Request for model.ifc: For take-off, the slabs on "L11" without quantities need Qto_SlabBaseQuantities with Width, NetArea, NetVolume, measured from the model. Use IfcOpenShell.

First a look at what the model holds.

```python
import ifcopenshell
import ifcopenshell.util.element
import ifcopenshell.util.unit

model = ifcopenshell.open("model.ifc")
print(model.schema)
for unit_type in ("LENGTHUNIT", "AREAUNIT", "VOLUMEUNIT"):
    print(unit_type, ifcopenshell.util.unit.calculate_unit_scale(model, unit_type))
storey = next(s for s in model.by_type("IfcBuildingStorey") if s.Name == "L11")
slabs = [e for e in ifcopenshell.util.element.get_decomposition(storey) if e.is_a("IfcSlab")]
for e in sorted(slabs, key=lambda e: e.id()):
    print(e.id(), e.is_a(), e.Name, list(ifcopenshell.util.element.get_psets(e, qtos_only=True)), sep=" | ")
```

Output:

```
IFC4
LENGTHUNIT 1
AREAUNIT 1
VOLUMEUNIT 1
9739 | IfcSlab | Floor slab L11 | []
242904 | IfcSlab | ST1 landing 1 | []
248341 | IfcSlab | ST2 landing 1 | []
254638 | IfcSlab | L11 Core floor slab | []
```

```python
import ifcopenshell
import ifcopenshell.api.pset
import ifcopenshell.geom
import ifcopenshell.util.element
import ifcopenshell.util.shape
import ifcopenshell.util.unit

model = ifcopenshell.open("model.ifc")
unit_scale = ifcopenshell.util.unit.calculate_unit_scale(model)
area_scale = ifcopenshell.util.unit.calculate_unit_scale(model, "AREAUNIT")
volume_scale = ifcopenshell.util.unit.calculate_unit_scale(model, "VOLUMEUNIT")
settings = ifcopenshell.geom.settings()

storey = next(s for s in model.by_type("IfcBuildingStorey") if s.Name == "L11")
slabs = [e for e in ifcopenshell.util.element.get_decomposition(storey) if e.is_a("IfcSlab")]

for e in sorted(slabs, key=lambda e: e.id()):
    if ifcopenshell.util.element.get_psets(e, qtos_only=True, should_inherit=False):
        continue
    # Geometry comes back in metres, in the element's own axes.
    shape = ifcopenshell.geom.create_shape(settings, e)
    values = {
        "Width": ifcopenshell.util.shape.get_z(shape.geometry) / unit_scale,
        "NetArea": ifcopenshell.util.shape.get_footprint_area(shape.geometry) / area_scale,
        "NetVolume": ifcopenshell.util.shape.get_volume(shape.geometry) / volume_scale,
    }
    qto = ifcopenshell.api.pset.add_qto(model, product=e, name="Qto_SlabBaseQuantities")
    ifcopenshell.api.pset.edit_qto(model, qto=qto, properties=values)
    print(e.id(), {k: round(v, 3) for k, v in values.items()})

model.write("model_rev.ifc")
```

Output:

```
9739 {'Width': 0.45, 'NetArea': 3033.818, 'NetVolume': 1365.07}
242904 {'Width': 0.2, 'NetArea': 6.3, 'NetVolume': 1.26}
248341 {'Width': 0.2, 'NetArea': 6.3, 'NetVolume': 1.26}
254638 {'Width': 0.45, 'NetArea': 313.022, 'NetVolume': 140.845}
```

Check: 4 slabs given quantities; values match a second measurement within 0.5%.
